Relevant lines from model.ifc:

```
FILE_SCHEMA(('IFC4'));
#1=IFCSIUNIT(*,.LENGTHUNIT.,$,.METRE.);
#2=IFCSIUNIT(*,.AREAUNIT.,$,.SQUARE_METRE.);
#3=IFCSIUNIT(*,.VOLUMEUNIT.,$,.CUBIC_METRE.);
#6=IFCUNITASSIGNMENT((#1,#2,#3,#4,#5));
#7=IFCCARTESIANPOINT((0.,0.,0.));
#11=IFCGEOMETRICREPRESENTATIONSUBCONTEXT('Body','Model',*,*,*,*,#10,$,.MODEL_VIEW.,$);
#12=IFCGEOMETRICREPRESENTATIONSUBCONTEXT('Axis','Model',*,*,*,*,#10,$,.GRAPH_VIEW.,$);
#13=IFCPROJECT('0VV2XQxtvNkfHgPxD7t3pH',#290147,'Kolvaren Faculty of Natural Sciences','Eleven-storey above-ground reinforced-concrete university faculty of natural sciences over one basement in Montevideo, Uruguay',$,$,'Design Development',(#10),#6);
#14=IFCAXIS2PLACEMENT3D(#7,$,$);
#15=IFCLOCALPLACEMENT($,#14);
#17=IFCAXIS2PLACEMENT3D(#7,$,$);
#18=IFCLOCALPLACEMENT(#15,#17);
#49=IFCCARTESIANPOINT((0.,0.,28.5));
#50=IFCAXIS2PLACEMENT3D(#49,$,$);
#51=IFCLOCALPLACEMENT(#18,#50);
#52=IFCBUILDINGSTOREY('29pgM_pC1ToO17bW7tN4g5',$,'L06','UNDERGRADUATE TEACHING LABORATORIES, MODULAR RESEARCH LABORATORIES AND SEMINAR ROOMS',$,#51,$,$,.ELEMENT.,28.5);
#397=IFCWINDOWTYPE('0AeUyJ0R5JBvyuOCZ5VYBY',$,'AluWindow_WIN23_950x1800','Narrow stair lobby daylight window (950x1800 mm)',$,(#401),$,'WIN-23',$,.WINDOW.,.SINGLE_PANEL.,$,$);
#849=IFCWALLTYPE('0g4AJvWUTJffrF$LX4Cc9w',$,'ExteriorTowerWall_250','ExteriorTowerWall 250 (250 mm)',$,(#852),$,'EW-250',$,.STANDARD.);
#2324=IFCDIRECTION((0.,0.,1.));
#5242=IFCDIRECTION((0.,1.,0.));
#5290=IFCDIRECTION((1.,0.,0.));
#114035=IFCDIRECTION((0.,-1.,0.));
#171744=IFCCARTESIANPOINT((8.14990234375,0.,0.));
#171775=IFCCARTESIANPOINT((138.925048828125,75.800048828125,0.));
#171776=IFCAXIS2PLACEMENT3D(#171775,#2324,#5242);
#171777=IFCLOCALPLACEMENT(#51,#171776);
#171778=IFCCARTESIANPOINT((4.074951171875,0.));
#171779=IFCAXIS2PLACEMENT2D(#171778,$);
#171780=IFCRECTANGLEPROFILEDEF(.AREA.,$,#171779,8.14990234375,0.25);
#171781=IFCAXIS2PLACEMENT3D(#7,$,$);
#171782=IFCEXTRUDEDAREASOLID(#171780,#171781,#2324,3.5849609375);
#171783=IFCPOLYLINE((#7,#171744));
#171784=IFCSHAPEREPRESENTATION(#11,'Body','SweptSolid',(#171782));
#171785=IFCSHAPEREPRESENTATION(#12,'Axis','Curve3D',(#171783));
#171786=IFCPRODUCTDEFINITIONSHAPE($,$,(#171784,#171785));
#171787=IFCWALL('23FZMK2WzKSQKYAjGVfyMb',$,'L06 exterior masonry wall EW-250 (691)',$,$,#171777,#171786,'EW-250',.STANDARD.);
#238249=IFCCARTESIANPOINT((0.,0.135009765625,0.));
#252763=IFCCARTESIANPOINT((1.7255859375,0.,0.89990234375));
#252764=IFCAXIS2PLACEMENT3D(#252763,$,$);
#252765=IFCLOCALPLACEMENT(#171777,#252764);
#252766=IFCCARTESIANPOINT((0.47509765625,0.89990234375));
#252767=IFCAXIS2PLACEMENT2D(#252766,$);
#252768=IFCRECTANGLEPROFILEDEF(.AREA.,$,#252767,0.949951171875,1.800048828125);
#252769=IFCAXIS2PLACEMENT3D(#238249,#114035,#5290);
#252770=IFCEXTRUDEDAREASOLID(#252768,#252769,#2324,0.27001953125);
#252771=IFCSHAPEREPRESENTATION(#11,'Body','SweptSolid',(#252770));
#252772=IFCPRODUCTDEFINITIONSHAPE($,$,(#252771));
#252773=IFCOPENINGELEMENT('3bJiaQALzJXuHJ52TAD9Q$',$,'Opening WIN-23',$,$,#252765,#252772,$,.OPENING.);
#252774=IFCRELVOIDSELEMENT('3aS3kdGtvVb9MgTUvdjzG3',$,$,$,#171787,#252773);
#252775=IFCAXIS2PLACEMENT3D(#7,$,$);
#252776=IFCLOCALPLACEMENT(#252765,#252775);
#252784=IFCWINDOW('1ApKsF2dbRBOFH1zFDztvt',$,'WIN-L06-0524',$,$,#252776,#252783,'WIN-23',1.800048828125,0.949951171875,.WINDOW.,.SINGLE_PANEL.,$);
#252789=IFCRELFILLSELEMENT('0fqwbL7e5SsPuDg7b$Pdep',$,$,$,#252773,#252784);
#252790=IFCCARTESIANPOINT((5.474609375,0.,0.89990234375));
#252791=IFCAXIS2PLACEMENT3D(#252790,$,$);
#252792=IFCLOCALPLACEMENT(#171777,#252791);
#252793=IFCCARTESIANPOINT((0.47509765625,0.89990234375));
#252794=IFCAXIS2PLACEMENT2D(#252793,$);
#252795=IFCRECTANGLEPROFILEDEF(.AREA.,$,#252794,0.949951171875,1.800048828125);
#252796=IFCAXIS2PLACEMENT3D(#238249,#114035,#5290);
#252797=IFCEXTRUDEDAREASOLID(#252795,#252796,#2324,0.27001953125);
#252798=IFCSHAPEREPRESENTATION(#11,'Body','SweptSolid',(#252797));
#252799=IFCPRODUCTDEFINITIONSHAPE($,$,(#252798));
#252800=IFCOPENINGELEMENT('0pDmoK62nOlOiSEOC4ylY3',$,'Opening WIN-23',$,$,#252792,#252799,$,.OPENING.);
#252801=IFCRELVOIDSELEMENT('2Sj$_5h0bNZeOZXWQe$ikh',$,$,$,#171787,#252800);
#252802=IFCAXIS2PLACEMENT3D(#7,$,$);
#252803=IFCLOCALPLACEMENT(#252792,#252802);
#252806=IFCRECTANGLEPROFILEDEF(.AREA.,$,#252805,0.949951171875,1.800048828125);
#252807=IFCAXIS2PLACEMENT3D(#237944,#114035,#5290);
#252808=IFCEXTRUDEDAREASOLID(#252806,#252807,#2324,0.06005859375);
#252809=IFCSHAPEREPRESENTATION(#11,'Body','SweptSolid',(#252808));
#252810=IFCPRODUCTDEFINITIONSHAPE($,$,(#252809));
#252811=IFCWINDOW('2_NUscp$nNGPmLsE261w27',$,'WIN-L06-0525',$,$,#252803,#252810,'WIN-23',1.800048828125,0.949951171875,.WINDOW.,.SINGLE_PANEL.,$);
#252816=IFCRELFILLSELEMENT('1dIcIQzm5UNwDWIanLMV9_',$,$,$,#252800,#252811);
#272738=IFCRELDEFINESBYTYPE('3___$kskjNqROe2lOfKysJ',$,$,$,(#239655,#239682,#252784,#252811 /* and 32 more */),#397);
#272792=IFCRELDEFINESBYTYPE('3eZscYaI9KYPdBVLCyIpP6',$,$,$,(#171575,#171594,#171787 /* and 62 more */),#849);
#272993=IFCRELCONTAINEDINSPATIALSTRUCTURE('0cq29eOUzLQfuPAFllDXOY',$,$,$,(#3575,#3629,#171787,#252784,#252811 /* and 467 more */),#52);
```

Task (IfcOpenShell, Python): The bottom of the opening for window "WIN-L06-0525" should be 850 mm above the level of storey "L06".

```python
import numpy as np
import ifcopenshell
import ifcopenshell.api.geometry
import ifcopenshell.geom
import ifcopenshell.util.element
import ifcopenshell.util.placement
import ifcopenshell.util.shape
import ifcopenshell.util.unit

model = ifcopenshell.open("model.ifc")
unit_scale = ifcopenshell.util.unit.calculate_unit_scale(model)

window = model.by_guid("2_NUscp$nNGPmLsE261w27")
opening = window.FillsVoids[0].RelatingOpeningElement
storey = ifcopenshell.util.element.get_container(window, ifc_class="IfcBuildingStorey")
level = ifcopenshell.util.placement.get_local_placement(storey.ObjectPlacement)[2, 3]

# The opening's origin need not be at the sill, so measure its lowest point.
shape = ifcopenshell.geom.create_shape(ifcopenshell.geom.settings(), opening)
bottom = ifcopenshell.util.shape.get_shape_bottom_elevation(shape, shape.geometry) / unit_scale
dz = level + 0.85 / unit_scale - bottom

shift = np.array([0.0, 0.0, dz])
# The window is placed relative to its opening, so it follows when the opening moves.
matrix = ifcopenshell.util.placement.get_local_placement(opening.ObjectPlacement)
matrix[:3, 3] += shift
ifcopenshell.api.geometry.edit_object_placement(
    model, product=opening, matrix=matrix, is_si=False, should_transform_children=True
)

print(f"moved by {dz * unit_scale:+.3f} m")

model.write("model-out.ifc")
```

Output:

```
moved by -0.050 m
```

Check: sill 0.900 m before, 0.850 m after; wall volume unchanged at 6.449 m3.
